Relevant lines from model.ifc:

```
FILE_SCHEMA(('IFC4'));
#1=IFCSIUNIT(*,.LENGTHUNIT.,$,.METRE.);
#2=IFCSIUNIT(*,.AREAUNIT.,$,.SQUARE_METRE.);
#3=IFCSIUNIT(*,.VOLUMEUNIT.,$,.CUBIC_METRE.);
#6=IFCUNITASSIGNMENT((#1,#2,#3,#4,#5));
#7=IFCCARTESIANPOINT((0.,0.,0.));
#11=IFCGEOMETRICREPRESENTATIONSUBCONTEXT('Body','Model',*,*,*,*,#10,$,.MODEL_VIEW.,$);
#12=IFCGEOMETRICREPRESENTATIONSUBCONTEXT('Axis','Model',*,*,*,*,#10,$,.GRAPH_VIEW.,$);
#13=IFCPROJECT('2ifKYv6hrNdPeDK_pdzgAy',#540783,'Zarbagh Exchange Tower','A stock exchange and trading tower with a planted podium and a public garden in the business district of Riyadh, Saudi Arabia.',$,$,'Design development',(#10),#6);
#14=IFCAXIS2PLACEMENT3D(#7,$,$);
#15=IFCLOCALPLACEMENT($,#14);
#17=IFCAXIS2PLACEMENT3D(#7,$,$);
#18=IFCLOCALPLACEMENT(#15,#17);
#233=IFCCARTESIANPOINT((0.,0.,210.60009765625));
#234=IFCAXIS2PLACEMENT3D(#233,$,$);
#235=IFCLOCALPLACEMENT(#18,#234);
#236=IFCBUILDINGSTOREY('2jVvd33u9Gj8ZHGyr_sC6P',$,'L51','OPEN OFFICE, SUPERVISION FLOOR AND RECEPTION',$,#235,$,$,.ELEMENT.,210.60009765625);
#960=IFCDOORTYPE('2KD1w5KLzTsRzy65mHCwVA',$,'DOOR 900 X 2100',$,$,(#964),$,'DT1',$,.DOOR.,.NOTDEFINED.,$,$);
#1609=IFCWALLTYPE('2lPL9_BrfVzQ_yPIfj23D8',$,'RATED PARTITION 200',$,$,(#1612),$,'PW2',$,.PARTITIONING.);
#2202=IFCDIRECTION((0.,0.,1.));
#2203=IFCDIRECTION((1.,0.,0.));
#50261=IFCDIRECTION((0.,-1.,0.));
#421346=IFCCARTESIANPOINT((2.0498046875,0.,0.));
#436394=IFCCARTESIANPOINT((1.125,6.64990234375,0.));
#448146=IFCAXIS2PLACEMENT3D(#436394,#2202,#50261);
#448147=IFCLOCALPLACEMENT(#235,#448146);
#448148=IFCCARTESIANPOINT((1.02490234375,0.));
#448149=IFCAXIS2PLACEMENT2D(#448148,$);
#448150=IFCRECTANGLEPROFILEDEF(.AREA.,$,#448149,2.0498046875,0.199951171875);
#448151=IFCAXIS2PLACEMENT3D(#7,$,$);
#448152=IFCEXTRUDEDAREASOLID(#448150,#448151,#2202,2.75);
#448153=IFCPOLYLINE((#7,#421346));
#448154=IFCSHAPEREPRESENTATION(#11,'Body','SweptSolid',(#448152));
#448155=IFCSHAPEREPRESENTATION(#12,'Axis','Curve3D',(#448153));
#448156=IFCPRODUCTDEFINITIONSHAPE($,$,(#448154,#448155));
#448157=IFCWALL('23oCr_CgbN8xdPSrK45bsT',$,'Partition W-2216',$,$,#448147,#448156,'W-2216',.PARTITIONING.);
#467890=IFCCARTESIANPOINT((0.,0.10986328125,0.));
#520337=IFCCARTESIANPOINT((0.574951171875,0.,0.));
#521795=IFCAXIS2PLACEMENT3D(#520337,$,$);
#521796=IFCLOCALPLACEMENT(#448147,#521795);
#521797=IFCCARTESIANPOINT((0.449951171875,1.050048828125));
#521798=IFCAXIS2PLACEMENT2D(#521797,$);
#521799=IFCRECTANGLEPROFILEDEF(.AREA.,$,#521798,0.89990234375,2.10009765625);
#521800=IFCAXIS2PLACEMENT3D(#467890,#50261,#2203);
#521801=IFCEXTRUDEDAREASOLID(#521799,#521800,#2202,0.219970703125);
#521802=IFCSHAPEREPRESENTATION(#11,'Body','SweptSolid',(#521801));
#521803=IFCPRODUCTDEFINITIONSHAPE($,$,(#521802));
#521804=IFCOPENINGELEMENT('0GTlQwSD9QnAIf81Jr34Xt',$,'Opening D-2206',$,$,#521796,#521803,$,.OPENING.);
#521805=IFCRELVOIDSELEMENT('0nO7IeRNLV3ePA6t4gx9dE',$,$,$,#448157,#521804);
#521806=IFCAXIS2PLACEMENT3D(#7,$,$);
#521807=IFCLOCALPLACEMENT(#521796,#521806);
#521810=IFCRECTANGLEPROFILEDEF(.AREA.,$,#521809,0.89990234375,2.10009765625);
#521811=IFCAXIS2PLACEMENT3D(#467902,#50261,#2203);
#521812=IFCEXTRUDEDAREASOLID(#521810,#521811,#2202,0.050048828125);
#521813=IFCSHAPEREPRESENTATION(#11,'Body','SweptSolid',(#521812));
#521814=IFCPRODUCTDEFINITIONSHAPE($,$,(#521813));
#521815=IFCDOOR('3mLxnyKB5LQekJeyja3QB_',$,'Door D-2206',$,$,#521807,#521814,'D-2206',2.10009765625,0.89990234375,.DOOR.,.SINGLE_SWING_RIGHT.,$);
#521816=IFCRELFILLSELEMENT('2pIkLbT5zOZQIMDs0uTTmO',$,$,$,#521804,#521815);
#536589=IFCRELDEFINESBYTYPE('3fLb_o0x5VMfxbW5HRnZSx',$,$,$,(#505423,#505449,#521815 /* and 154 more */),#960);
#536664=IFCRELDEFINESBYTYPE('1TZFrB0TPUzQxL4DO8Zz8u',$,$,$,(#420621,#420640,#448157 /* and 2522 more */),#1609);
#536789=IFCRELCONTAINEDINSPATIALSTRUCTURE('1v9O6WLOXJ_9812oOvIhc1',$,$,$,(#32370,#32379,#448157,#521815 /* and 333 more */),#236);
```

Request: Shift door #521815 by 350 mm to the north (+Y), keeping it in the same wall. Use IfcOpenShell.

```python
import ifcopenshell
import ifcopenshell.api.geometry
import ifcopenshell.util.placement

model = ifcopenshell.open("model.ifc")

door = model.by_guid("3mLxnyKB5LQekJeyja3QB_")
opening = door.FillsVoids[0].RelatingOpeningElement
wall = opening.VoidsElements[0].RelatingBuildingElement

wall_matrix = ifcopenshell.util.placement.get_local_placement(wall.ObjectPlacement)
shift = wall_matrix[:3, 0] * -0.35
before = ifcopenshell.util.placement.get_local_placement(door.ObjectPlacement)[:3, 3].copy()

# The door is placed relative to its opening, so it follows when the opening moves.
matrix = ifcopenshell.util.placement.get_local_placement(opening.ObjectPlacement)
matrix[:3, 3] += shift
ifcopenshell.api.geometry.edit_object_placement(
    model, product=opening, matrix=matrix, is_si=False, should_transform_children=True
)

after = ifcopenshell.util.placement.get_local_placement(door.ObjectPlacement)[:3, 3]
print("door moved by", (after - before).round(3) + 0.0)

model.write("model_edited.ifc")
```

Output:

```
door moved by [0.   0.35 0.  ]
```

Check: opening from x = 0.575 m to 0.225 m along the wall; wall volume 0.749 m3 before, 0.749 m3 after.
